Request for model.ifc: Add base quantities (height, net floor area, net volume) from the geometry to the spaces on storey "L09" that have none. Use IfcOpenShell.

First a look at what the model holds.

```python
import ifcopenshell
import ifcopenshell.util.element
import ifcopenshell.util.unit

model = ifcopenshell.open("model.ifc")
print(model.schema)
for unit_type in ("LENGTHUNIT", "AREAUNIT", "VOLUMEUNIT"):
    print(unit_type, ifcopenshell.util.unit.calculate_unit_scale(model, unit_type))
storey = next(s for s in model.by_type("IfcBuildingStorey") if s.Name == "L09")
spaces = [e for e in ifcopenshell.util.element.get_decomposition(storey) if e.is_a("IfcSpace")]
for e in sorted(spaces, key=lambda e: e.id()):
    print(e.id(), e.is_a(), e.Name, list(ifcopenshell.util.element.get_psets(e, qtos_only=True)), sep=" | ")
```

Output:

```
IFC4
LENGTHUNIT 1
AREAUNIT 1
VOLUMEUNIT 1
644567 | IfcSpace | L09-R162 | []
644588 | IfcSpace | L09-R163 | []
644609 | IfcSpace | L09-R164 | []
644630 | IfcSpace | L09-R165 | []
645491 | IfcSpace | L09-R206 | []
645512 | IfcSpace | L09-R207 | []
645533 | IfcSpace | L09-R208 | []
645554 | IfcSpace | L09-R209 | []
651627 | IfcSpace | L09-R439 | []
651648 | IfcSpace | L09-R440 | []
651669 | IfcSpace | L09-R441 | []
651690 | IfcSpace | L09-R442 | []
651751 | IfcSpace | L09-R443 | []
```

```python
import ifcopenshell
import ifcopenshell.api.pset
import ifcopenshell.geom
import ifcopenshell.util.element
import ifcopenshell.util.shape
import ifcopenshell.util.unit

model = ifcopenshell.open("model.ifc")
unit_scale = ifcopenshell.util.unit.calculate_unit_scale(model)
area_scale = ifcopenshell.util.unit.calculate_unit_scale(model, "AREAUNIT")
volume_scale = ifcopenshell.util.unit.calculate_unit_scale(model, "VOLUMEUNIT")
settings = ifcopenshell.geom.settings()

storey = next(s for s in model.by_type("IfcBuildingStorey") if s.Name == "L09")
spaces = [e for e in ifcopenshell.util.element.get_decomposition(storey) if e.is_a("IfcSpace")]

for e in sorted(spaces, key=lambda e: e.id()):
    if ifcopenshell.util.element.get_psets(e, qtos_only=True, should_inherit=False):
        continue
    # Geometry comes back in metres, in the element's own axes.
    shape = ifcopenshell.geom.create_shape(settings, e)
    values = {
        "Height": ifcopenshell.util.shape.get_z(shape.geometry) / unit_scale,
        "NetFloorArea": ifcopenshell.util.shape.get_footprint_area(shape.geometry) / area_scale,
        "NetVolume": ifcopenshell.util.shape.get_volume(shape.geometry) / volume_scale,
    }
    qto = ifcopenshell.api.pset.add_qto(model, product=e, name="Qto_SpaceBaseQuantities")
    ifcopenshell.api.pset.edit_qto(model, qto=qto, properties=values)
    print(e.id(), {k: round(v, 3) for k, v in values.items()})

model.write("model_v2.ifc")
```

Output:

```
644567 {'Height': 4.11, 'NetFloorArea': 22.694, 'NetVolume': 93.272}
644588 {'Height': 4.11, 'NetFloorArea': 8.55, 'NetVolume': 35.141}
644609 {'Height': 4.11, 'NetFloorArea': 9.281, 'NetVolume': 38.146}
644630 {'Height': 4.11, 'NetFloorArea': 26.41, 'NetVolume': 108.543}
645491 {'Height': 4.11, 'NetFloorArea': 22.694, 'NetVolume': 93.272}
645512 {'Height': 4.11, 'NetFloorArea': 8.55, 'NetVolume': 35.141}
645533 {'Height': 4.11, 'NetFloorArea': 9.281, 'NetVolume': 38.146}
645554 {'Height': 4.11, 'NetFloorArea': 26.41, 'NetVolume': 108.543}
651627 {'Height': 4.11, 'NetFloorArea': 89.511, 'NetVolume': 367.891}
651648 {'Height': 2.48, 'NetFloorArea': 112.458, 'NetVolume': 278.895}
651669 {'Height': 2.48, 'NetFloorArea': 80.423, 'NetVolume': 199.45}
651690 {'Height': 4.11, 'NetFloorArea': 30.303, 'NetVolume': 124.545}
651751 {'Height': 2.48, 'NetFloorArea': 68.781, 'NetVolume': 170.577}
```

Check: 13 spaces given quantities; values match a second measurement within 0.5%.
